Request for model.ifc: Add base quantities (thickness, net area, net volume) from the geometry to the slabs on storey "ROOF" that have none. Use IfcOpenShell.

First a look at what the model holds.

```python
import ifcopenshell
import ifcopenshell.util.element
import ifcopenshell.util.unit

model = ifcopenshell.open("model.ifc")
print(model.schema)
for unit_type in ("LENGTHUNIT", "AREAUNIT", "VOLUMEUNIT"):
    print(unit_type, ifcopenshell.util.unit.calculate_unit_scale(model, unit_type))
storey = next(s for s in model.by_type("IfcBuildingStorey") if s.Name == "ROOF")
slabs = [e for e in ifcopenshell.util.element.get_decomposition(storey) if e.is_a("IfcSlab")]
for e in sorted(slabs, key=lambda e: e.id()):
    print(e.id(), e.is_a(), e.Name, list(ifcopenshell.util.element.get_psets(e, qtos_only=True)), sep=" | ")
```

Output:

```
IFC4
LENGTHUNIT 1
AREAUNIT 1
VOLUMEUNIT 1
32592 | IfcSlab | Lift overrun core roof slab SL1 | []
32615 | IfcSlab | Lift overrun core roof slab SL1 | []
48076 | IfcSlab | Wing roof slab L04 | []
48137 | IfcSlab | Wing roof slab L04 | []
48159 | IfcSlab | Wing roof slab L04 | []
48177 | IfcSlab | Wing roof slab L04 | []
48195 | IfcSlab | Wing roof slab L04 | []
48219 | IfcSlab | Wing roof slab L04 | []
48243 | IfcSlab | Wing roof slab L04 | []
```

```python
import ifcopenshell
import ifcopenshell.api.pset
import ifcopenshell.geom
import ifcopenshell.util.element
import ifcopenshell.util.shape
import ifcopenshell.util.unit

model = ifcopenshell.open("model.ifc")
unit_scale = ifcopenshell.util.unit.calculate_unit_scale(model)
area_scale = ifcopenshell.util.unit.calculate_unit_scale(model, "AREAUNIT")
volume_scale = ifcopenshell.util.unit.calculate_unit_scale(model, "VOLUMEUNIT")
settings = ifcopenshell.geom.settings()

storey = next(s for s in model.by_type("IfcBuildingStorey") if s.Name == "ROOF")
slabs = [e for e in ifcopenshell.util.element.get_decomposition(storey) if e.is_a("IfcSlab")]

for e in sorted(slabs, key=lambda e: e.id()):
    if ifcopenshell.util.element.get_psets(e, qtos_only=True, should_inherit=False):
        continue
    # Geometry comes back in metres, in the element's own axes.
    shape = ifcopenshell.geom.create_shape(settings, e)
    values = {
        "Width": ifcopenshell.util.shape.get_z(shape.geometry) / unit_scale,
        "NetArea": ifcopenshell.util.shape.get_footprint_area(shape.geometry) / area_scale,
        "NetVolume": ifcopenshell.util.shape.get_volume(shape.geometry) / volume_scale,
    }
    qto = ifcopenshell.api.pset.add_qto(model, product=e, name="Qto_SlabBaseQuantities")
    ifcopenshell.api.pset.edit_qto(model, qto=qto, properties=values)
    print(e.id(), {k: round(v, 3) for k, v in values.items()})

model.write("model_rev.ifc")
```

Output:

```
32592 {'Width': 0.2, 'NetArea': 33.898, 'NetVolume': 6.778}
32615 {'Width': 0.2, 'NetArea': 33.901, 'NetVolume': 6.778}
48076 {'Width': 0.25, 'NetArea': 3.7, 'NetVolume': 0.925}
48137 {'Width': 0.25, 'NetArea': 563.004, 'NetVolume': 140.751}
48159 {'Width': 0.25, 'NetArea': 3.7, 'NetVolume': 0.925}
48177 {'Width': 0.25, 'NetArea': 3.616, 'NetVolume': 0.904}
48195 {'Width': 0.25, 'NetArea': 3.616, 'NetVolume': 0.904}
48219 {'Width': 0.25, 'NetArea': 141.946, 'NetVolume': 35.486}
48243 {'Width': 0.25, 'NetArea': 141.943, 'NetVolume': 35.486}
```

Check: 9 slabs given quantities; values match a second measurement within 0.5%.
